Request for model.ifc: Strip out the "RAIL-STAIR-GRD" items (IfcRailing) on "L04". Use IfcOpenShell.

First a look at what the model holds.

```python
import ifcopenshell
import ifcopenshell.util.element

model = ifcopenshell.open("model.ifc")
print(model.schema)
storey = next(s for s in model.by_type("IfcBuildingStorey") if s.Name == "L04")
railings = [e for e in ifcopenshell.util.element.get_decomposition(storey) if e.is_a("IfcRailing")]
seen = {}
for e in railings:
    element_type = ifcopenshell.util.element.get_type(e)
    name = element_type.Name if element_type not in (None, e) else None
    seen[name] = seen.get(name, 0) + 1
for name, count in sorted(seen.items(), key=str):
    print(count, "x", name)
```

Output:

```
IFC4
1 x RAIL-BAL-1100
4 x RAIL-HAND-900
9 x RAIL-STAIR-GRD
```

```python
import ifcopenshell
import ifcopenshell.api.root
import ifcopenshell.util.element

model = ifcopenshell.open("model.ifc")

storey = next(s for s in model.by_type("IfcBuildingStorey") if s.Name == "L04")
railings = [e for e in ifcopenshell.util.element.get_decomposition(storey) if e.is_a("IfcRailing")]
targets = [e for e in railings if (t := ifcopenshell.util.element.get_type(e)) not in (None, e) and t.Name == "RAIL-STAIR-GRD"]

for e in targets:
    ifcopenshell.api.root.remove_product(model, product=e)
print(len(targets), "removed")

model.write("model_edited.ifc")
```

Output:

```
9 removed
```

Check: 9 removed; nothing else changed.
